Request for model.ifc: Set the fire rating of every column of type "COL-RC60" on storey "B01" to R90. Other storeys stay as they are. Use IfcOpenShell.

First a look at what the model holds.

```python
import ifcopenshell
import ifcopenshell.util.element

model = ifcopenshell.open("model.ifc")
print(model.schema)
storey = next(s for s in model.by_type("IfcBuildingStorey") if s.Name == "B01")
columns = [e for e in ifcopenshell.util.element.get_decomposition(storey) if e.is_a("IfcColumn")]
seen = {}
for e in columns:
    element_type = ifcopenshell.util.element.get_type(e)
    key = (element_type.Name if element_type != e and element_type else None, ifcopenshell.util.element.get_pset(e, "Pset_ColumnCommon", "FireRating"))
    seen[key] = seen.get(key, 0) + 1
for (name, value), count in sorted(seen.items(), key=str):
    print(count, "x", name, "|", value)
```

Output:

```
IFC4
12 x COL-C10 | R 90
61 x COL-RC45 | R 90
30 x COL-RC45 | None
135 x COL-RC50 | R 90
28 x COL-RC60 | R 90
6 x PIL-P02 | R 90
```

```python
import ifcopenshell
import ifcopenshell.api.pset
import ifcopenshell.util.element

model = ifcopenshell.open("model.ifc")

storey = next(s for s in model.by_type("IfcBuildingStorey") if s.Name == "B01")
columns = [e for e in ifcopenshell.util.element.get_decomposition(storey) if e.is_a("IfcColumn")]

count = 0
for e in columns:
    element_type = ifcopenshell.util.element.get_type(e)
    if element_type in (None, e) or element_type.Name != "COL-RC60":
        continue
    # add_pset returns the element's existing set when there is one.
    pset = ifcopenshell.api.pset.add_pset(model, product=e, name="Pset_ColumnCommon")
    ifcopenshell.api.pset.edit_pset(model, pset=pset, properties={"FireRating": "R90"})
    count += 1

print(count, "columns updated")

model.write("model_updated.ifc")
```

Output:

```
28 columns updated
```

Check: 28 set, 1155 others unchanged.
